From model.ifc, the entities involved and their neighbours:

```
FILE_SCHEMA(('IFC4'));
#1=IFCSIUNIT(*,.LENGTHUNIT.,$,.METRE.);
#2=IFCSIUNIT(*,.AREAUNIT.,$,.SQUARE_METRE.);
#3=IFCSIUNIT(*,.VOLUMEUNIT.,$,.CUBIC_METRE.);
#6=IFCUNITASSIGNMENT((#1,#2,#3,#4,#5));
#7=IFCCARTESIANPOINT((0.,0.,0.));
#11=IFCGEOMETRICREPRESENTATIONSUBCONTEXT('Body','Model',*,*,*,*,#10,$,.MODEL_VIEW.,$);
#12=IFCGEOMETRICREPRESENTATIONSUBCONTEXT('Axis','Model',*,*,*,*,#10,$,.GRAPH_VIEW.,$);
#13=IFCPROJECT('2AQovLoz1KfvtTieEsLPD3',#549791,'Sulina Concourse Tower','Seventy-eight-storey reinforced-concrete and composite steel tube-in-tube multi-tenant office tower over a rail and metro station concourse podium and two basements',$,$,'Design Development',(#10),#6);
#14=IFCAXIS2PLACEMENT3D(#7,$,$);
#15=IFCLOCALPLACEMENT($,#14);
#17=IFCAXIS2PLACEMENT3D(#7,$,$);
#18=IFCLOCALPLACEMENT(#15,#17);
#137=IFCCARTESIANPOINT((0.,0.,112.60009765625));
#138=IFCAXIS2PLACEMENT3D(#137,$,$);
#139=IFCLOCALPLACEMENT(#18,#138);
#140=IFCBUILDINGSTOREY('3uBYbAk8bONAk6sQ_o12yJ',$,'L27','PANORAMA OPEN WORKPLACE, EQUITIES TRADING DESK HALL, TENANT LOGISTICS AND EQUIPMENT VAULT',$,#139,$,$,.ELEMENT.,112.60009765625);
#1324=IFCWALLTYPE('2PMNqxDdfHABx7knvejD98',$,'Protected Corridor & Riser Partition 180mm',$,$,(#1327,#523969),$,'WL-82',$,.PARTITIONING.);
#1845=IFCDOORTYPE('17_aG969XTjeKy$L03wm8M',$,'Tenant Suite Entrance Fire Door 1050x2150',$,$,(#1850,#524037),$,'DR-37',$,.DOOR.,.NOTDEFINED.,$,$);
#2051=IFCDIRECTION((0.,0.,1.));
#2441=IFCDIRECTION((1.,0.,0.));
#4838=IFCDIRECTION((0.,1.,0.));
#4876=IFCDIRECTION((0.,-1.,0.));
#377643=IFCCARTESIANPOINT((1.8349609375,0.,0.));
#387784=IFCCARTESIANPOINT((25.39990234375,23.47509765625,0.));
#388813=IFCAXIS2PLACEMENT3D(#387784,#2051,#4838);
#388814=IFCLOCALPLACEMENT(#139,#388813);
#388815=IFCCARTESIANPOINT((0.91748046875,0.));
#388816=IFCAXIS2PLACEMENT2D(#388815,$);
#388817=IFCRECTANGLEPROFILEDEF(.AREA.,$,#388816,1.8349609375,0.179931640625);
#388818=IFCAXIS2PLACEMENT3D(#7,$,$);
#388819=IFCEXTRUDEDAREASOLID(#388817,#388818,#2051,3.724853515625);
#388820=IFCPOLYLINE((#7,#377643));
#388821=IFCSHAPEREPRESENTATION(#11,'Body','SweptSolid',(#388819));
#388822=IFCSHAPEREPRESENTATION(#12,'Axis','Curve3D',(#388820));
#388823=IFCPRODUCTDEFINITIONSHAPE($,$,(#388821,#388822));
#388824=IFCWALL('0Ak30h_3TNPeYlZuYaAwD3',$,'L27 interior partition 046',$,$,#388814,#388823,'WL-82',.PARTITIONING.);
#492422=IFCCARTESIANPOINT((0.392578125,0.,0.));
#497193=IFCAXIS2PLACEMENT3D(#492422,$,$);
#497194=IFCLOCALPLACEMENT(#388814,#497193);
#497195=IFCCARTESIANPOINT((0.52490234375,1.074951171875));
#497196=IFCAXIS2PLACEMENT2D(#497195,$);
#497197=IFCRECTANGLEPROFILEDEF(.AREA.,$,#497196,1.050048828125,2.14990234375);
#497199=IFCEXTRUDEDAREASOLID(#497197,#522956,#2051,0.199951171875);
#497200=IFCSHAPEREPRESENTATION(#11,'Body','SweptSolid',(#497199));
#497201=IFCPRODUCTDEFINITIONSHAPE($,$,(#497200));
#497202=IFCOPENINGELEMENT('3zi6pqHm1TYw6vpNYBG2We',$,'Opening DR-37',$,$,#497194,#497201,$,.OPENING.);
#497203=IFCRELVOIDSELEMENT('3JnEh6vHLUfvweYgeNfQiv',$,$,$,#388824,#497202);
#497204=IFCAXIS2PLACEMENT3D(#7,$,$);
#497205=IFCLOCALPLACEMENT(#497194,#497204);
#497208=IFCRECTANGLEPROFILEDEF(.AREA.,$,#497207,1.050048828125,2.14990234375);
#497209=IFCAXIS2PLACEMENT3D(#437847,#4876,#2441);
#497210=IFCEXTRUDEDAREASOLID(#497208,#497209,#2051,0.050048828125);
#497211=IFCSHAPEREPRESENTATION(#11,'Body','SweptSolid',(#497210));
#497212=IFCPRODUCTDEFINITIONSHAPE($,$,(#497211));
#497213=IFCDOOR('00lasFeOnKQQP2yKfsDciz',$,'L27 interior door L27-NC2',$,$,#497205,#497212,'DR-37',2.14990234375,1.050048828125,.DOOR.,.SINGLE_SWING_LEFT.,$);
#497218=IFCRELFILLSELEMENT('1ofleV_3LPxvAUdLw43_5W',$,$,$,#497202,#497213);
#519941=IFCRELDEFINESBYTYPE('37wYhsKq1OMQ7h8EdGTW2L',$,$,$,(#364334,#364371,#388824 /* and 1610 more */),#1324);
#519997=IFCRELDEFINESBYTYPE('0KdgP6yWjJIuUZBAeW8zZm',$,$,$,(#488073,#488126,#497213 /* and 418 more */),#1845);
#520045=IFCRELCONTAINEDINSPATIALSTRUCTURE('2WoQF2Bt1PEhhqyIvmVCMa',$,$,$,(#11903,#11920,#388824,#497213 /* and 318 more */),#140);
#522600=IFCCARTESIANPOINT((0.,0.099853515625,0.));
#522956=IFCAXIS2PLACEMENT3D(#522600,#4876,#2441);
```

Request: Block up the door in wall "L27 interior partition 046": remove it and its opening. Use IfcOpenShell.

```python
import ifcopenshell
import ifcopenshell.api.feature
import ifcopenshell.api.root
import ifcopenshell.geom
import ifcopenshell.util.shape

model = ifcopenshell.open("model.ifc")
settings = ifcopenshell.geom.settings()


def volume(element):
    """Net volume in cubic metres, openings subtracted."""
    shape = ifcopenshell.geom.create_shape(settings, element)
    return ifcopenshell.util.shape.get_volume(shape.geometry)


door = model.by_guid("00lasFeOnKQQP2yKfsDciz")
opening = door.FillsVoids[0].RelatingOpeningElement
wall = opening.VoidsElements[0].RelatingBuildingElement
before = volume(wall)

ifcopenshell.api.root.remove_product(model, product=door)
ifcopenshell.api.feature.remove_feature(model, feature=opening)

after = volume(wall)

print(f"wall volume {before:.3f} -> {after:.3f} m3")

model.write("model_v2.ifc")
```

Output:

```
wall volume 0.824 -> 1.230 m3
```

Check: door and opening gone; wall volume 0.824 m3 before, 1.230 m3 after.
